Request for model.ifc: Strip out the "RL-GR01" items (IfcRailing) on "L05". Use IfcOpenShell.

First a look at what the model holds.

```python
import ifcopenshell
import ifcopenshell.util.element

model = ifcopenshell.open("model.ifc")
print(model.schema)
storey = next(s for s in model.by_type("IfcBuildingStorey") if s.Name == "L05")
railings = [e for e in ifcopenshell.util.element.get_decomposition(storey) if e.is_a("IfcRailing")]
seen = {}
for e in railings:
    element_type = ifcopenshell.util.element.get_type(e)
    name = element_type.Name if element_type not in (None, e) else None
    seen[name] = seen.get(name, 0) + 1
for name, count in sorted(seen.items(), key=str):
    print(count, "x", name)
```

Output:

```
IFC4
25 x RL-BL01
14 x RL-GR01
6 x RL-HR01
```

```python
import ifcopenshell
import ifcopenshell.api.root
import ifcopenshell.util.element

model = ifcopenshell.open("model.ifc")

storey = next(s for s in model.by_type("IfcBuildingStorey") if s.Name == "L05")
railings = [e for e in ifcopenshell.util.element.get_decomposition(storey) if e.is_a("IfcRailing")]
targets = [e for e in railings if (t := ifcopenshell.util.element.get_type(e)) not in (None, e) and t.Name == "RL-GR01"]

for e in targets:
    ifcopenshell.api.root.remove_product(model, product=e)
print(len(targets), "removed")

model.write("model_edited.ifc")
```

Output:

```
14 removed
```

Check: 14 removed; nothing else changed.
